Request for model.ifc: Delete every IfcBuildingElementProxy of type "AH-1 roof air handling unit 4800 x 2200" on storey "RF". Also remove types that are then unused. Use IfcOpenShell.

First a look at what the model holds.

```python
import ifcopenshell
import ifcopenshell.util.element

model = ifcopenshell.open("model.ifc")
print(model.schema)
storey = next(s for s in model.by_type("IfcBuildingStorey") if s.Name == "RF")
proxies = [e for e in ifcopenshell.util.element.get_decomposition(storey) if e.is_a("IfcBuildingElementProxy")]
seen = {}
for e in proxies:
    element_type = ifcopenshell.util.element.get_type(e)
    name = element_type.Name if element_type not in (None, e) else None
    seen[name] = seen.get(name, 0) + 1
for name, count in sorted(seen.items(), key=str):
    print(count, "x", name)
```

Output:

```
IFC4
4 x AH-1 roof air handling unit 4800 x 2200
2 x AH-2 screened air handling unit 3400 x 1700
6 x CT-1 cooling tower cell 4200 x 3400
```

```python
import ifcopenshell
import ifcopenshell.api.root
import ifcopenshell.util.element

model = ifcopenshell.open("model.ifc")

storey = next(s for s in model.by_type("IfcBuildingStorey") if s.Name == "RF")
proxies = [e for e in ifcopenshell.util.element.get_decomposition(storey) if e.is_a("IfcBuildingElementProxy")]
targets = [e for e in proxies if (t := ifcopenshell.util.element.get_type(e)) not in (None, e) and t.Name == "AH-1 roof air handling unit 4800 x 2200"]
types = {ifcopenshell.util.element.get_type(e) for e in targets} - {None, *targets}

for e in targets:
    ifcopenshell.api.root.remove_product(model, product=e)
print(len(targets), "removed")

unused = [t for t in types if not ifcopenshell.util.element.get_types(t)]
for t in unused:
    ifcopenshell.api.root.remove_product(model, product=t)
print(len(unused), "unused types removed")

model.write("model_v2.ifc")
```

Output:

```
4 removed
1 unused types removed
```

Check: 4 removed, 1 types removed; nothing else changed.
